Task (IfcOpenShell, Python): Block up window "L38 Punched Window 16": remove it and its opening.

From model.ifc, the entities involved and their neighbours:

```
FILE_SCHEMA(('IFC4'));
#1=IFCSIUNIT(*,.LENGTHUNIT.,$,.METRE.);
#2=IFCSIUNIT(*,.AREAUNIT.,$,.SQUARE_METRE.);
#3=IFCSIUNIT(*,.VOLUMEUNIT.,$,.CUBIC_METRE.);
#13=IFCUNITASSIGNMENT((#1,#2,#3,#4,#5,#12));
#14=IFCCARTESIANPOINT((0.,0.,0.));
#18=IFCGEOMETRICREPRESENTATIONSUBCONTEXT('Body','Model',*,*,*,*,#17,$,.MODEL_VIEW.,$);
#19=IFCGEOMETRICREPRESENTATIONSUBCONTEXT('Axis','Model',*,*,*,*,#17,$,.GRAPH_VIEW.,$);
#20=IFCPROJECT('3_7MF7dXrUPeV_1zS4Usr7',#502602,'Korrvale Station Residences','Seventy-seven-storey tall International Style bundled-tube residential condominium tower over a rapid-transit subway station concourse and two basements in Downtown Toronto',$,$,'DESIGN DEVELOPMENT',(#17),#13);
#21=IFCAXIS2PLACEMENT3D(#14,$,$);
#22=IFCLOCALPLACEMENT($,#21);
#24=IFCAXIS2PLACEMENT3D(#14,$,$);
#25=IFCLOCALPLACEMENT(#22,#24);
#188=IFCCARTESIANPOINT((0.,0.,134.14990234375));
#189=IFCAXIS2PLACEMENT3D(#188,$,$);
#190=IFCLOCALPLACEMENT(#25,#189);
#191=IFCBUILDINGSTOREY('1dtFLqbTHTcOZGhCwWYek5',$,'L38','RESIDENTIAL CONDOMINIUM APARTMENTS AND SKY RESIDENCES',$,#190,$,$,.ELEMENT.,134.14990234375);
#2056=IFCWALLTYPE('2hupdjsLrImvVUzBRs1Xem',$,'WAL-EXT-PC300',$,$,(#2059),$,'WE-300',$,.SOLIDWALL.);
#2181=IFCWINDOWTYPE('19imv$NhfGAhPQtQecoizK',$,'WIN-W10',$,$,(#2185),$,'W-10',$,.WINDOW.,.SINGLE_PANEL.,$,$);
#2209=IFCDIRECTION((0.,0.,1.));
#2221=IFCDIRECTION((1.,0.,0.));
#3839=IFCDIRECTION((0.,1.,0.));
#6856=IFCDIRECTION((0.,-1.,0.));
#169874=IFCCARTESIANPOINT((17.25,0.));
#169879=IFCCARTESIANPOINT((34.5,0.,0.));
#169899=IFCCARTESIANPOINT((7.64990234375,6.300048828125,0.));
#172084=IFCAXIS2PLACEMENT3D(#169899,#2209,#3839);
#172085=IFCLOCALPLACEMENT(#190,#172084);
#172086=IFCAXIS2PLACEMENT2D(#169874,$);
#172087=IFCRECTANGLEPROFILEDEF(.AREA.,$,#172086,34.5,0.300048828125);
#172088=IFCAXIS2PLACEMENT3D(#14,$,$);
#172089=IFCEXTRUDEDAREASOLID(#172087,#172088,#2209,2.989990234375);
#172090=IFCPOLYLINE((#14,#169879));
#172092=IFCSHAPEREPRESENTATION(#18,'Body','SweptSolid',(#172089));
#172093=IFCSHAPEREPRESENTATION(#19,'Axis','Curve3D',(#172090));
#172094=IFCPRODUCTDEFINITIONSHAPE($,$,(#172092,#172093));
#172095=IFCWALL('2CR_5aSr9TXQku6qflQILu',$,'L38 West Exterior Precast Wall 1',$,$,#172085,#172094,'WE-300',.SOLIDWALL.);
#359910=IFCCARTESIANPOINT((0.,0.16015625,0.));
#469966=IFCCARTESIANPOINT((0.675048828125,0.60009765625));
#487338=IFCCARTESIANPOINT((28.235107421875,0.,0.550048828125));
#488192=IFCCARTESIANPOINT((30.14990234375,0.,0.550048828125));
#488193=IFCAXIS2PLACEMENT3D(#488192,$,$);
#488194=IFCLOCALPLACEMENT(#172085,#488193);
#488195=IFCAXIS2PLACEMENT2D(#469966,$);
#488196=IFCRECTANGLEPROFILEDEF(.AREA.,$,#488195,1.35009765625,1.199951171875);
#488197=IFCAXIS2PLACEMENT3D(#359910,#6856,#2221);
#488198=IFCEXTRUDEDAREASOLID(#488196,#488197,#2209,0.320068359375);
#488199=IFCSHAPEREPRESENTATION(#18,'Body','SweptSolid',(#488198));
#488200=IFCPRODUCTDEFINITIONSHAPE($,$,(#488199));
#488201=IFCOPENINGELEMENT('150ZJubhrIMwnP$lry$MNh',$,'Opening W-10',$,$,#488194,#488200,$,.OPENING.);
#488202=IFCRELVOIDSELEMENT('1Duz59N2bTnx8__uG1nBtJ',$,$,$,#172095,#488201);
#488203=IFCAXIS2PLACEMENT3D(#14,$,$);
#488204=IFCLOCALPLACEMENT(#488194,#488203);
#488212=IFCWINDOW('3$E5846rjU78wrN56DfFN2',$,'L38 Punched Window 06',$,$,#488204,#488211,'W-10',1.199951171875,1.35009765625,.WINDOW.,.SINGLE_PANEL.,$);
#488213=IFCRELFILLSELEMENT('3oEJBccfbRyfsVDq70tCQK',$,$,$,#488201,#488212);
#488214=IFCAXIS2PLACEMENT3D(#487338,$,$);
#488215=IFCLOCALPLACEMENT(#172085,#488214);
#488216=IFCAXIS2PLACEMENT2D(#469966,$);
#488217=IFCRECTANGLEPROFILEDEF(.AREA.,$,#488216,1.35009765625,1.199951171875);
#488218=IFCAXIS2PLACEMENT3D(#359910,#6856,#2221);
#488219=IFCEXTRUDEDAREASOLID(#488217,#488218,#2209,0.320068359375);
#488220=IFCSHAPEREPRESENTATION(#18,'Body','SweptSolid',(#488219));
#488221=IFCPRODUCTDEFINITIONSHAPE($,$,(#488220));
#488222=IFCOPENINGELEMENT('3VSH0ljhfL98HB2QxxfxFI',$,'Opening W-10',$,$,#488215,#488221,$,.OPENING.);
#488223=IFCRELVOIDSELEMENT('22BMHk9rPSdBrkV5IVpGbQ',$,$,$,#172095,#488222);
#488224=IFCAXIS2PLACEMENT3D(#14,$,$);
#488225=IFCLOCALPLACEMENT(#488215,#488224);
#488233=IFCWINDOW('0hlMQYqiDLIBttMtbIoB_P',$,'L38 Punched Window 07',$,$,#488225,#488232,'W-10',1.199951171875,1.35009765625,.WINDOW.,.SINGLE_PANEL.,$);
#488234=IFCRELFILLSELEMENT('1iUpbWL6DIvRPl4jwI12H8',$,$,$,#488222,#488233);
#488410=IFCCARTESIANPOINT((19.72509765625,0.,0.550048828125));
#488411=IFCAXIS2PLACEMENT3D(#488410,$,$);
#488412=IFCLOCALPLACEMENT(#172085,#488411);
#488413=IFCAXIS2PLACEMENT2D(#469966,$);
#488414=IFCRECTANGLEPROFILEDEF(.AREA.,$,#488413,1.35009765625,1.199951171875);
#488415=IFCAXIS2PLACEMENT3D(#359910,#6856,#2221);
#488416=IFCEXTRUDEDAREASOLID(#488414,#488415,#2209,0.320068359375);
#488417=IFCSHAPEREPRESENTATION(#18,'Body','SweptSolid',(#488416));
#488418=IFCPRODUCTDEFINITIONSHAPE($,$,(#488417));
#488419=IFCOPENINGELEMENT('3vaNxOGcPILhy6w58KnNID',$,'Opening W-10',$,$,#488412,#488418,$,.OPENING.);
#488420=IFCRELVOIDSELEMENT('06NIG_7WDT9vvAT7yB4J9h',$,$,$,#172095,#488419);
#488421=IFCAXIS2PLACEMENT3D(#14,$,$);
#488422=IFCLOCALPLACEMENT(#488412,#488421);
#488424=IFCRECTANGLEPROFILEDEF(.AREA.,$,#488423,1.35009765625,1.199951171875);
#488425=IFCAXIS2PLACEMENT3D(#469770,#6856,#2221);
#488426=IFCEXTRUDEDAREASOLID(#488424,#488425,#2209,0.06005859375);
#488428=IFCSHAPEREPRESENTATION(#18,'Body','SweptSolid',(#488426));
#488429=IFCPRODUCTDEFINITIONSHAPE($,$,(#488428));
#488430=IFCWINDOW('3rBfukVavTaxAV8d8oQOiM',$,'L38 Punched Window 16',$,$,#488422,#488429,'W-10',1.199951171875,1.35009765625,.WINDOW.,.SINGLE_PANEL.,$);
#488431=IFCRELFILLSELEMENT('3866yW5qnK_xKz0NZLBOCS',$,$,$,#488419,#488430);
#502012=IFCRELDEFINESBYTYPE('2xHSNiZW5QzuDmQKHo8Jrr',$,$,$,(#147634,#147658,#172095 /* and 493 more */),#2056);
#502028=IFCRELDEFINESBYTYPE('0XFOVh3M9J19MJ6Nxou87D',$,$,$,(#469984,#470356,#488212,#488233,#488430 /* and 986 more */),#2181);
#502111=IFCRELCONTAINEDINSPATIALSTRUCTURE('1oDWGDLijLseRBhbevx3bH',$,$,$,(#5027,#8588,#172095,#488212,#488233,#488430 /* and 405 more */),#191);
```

```python
import ifcopenshell
import ifcopenshell.api.feature
import ifcopenshell.api.root
import ifcopenshell.geom
import ifcopenshell.util.shape

model = ifcopenshell.open("model.ifc")
settings = ifcopenshell.geom.settings()


def volume(element):
    """Net volume in cubic metres, openings subtracted."""
    shape = ifcopenshell.geom.create_shape(settings, element)
    return ifcopenshell.util.shape.get_volume(shape.geometry)


window = model.by_id(488430)
opening = window.FillsVoids[0].RelatingOpeningElement
wall = opening.VoidsElements[0].RelatingBuildingElement
before = volume(wall)

ifcopenshell.api.root.remove_product(model, product=window)
ifcopenshell.api.feature.remove_feature(model, feature=opening)

after = volume(wall)

print(f"wall volume {before:.3f} -> {after:.3f} m3")

model.write("model_updated.ifc")
```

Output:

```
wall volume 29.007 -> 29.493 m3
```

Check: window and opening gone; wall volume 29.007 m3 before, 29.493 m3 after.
